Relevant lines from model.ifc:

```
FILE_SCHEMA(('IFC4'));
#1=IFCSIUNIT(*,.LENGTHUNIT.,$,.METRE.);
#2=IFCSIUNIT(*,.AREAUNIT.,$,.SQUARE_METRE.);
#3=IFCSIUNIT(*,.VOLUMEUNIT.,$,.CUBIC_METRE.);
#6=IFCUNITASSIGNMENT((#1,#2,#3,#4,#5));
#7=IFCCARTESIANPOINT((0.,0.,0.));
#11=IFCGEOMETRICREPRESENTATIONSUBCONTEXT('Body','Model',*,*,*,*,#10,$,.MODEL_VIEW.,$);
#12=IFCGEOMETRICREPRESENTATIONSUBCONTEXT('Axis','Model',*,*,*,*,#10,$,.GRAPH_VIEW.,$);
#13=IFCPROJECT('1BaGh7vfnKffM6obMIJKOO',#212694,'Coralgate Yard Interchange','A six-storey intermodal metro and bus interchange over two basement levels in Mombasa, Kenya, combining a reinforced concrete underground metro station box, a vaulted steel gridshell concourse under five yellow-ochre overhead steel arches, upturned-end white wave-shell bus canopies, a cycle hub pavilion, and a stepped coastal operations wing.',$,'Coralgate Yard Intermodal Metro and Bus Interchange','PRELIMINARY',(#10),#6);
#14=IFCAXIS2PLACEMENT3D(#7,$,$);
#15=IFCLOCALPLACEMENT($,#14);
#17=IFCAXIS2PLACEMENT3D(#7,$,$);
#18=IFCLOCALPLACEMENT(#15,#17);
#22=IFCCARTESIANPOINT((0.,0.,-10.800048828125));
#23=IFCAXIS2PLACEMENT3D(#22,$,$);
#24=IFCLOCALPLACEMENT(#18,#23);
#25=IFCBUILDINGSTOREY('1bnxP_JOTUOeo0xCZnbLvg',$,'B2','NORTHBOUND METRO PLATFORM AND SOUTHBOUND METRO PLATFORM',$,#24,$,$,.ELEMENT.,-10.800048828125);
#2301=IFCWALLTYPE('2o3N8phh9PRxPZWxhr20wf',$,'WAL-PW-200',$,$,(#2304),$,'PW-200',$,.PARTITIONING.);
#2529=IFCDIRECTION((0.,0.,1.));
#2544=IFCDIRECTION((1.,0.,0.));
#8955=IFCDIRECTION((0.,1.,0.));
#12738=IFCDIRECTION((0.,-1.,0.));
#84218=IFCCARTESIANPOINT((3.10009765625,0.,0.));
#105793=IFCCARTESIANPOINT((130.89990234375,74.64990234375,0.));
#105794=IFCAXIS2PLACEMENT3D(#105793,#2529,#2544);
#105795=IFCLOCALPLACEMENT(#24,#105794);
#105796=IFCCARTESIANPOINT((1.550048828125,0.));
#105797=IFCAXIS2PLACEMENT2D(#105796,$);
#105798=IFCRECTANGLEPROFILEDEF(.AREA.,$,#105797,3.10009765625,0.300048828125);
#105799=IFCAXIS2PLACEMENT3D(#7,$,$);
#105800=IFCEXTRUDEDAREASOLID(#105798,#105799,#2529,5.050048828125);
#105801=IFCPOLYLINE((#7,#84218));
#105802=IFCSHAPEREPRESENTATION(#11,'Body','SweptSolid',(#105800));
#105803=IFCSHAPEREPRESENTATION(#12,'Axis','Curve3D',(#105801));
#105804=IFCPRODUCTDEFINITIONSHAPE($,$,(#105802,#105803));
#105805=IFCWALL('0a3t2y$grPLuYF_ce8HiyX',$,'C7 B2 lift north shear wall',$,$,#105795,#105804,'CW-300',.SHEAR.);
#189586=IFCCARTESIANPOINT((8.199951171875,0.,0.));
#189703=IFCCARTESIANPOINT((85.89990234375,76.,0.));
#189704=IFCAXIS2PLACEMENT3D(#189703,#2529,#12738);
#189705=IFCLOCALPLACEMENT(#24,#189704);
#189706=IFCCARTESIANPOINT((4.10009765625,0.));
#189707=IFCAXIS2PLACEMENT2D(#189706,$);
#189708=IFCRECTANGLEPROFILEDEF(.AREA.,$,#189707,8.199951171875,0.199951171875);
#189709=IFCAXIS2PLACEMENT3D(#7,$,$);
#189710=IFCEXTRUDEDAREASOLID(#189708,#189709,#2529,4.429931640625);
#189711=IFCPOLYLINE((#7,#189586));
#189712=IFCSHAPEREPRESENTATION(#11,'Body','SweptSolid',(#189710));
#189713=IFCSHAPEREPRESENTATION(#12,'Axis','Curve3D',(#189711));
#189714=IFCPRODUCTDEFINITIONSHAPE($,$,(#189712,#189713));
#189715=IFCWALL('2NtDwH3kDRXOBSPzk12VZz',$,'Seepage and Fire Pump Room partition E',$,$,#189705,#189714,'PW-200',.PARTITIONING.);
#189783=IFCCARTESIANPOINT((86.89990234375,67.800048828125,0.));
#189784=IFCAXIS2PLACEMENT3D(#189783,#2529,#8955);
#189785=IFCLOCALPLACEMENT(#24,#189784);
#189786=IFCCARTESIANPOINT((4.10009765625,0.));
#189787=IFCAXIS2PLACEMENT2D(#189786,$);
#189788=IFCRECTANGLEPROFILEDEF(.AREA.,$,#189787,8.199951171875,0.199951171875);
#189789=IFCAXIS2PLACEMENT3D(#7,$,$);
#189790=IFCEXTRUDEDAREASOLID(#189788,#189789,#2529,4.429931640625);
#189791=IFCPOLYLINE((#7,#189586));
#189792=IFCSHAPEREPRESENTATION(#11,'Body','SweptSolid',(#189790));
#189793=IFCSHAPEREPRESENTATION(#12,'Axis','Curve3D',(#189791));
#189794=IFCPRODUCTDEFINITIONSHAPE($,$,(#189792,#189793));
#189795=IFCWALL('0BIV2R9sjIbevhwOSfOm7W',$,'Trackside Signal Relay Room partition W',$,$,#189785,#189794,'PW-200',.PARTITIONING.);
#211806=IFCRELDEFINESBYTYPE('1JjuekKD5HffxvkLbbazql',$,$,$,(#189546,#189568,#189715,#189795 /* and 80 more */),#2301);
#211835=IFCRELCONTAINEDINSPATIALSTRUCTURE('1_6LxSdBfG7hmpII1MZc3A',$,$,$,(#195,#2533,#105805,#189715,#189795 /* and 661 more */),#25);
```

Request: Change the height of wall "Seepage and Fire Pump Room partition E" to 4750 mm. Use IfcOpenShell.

```python
import ifcopenshell
import ifcopenshell.geom
import ifcopenshell.util.representation
import ifcopenshell.util.shape

model = ifcopenshell.open("model.ifc")
settings = ifcopenshell.geom.settings()


def volume(element):
    """Net volume in cubic metres, openings subtracted."""
    shape = ifcopenshell.geom.create_shape(settings, element)
    return ifcopenshell.util.shape.get_volume(shape.geometry)


wall = model.by_guid("2NtDwH3kDRXOBSPzk12VZz")
before = volume(wall)

body = ifcopenshell.util.representation.get_representation(wall, "Model", "Body")
solid = body.Items[0]
old_height = solid.Depth
solid.Depth = 4.75
after = volume(wall)

print(f"height {old_height:g} -> {solid.Depth:g}, volume {before:.3f} -> {after:.3f} m3")

model.write("model_updated.ifc")
```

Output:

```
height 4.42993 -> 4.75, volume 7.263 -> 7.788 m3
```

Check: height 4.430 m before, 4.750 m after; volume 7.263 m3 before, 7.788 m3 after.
